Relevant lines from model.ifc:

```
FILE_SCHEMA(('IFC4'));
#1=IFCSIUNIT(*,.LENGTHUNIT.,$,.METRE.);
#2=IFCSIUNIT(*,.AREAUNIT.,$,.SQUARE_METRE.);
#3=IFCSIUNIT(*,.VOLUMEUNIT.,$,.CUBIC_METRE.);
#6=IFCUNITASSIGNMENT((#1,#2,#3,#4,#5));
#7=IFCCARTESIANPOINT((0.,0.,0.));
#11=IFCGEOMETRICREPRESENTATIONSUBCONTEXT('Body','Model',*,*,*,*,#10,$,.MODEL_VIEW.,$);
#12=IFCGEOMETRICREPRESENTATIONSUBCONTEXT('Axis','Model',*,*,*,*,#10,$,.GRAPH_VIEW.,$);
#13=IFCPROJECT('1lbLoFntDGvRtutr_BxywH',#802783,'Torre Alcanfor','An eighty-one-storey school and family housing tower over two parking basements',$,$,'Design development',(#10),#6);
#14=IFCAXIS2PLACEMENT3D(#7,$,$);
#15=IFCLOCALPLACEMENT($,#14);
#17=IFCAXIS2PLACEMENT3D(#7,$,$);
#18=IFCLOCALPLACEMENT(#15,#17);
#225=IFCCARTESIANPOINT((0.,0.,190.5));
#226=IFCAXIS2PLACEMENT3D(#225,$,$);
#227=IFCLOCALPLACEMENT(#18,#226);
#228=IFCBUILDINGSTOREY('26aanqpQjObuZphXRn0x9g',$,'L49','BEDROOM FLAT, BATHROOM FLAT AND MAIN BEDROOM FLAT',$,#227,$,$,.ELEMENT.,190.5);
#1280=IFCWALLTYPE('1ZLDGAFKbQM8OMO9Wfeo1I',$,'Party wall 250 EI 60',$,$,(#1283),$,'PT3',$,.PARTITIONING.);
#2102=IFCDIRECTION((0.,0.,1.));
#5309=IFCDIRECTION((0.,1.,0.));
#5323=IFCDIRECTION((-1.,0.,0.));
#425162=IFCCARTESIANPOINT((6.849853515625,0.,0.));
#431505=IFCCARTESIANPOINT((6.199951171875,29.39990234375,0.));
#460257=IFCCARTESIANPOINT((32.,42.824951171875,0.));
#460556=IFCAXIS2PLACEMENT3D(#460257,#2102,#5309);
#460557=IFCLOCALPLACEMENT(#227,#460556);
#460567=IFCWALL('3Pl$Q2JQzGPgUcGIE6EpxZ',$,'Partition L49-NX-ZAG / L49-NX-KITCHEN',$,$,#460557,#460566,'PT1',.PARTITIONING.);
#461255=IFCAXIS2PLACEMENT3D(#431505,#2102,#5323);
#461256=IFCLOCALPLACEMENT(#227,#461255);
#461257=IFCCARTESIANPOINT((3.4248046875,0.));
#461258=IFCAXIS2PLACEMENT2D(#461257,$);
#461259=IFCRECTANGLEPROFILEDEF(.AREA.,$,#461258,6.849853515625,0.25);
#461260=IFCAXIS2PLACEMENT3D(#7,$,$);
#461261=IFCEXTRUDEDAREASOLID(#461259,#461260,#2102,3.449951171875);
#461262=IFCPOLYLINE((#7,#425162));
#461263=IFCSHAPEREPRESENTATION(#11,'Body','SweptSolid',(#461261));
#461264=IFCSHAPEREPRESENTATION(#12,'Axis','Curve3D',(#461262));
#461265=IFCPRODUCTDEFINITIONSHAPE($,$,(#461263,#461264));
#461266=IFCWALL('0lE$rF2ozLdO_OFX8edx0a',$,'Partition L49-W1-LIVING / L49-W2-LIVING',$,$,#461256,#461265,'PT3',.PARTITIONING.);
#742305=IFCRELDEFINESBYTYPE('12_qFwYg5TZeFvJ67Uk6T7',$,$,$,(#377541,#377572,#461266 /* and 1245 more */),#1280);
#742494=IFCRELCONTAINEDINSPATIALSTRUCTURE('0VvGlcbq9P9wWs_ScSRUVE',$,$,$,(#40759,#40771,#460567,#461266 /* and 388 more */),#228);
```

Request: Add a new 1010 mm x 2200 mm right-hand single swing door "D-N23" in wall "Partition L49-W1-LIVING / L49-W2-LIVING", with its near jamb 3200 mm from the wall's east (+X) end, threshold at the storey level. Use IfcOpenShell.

```python
import numpy as np
import ifcopenshell
import ifcopenshell.api.feature
import ifcopenshell.api.geometry
import ifcopenshell.api.root
import ifcopenshell.api.spatial
import ifcopenshell.geom
import ifcopenshell.util.element
import ifcopenshell.util.placement
import ifcopenshell.util.representation
import ifcopenshell.util.shape
import ifcopenshell.util.unit

model = ifcopenshell.open("model.ifc")
unit_scale = ifcopenshell.util.unit.calculate_unit_scale(model)
settings = ifcopenshell.geom.settings()


def volume(element):
    """Net volume in cubic metres, openings subtracted."""
    shape = ifcopenshell.geom.create_shape(settings, element)
    return ifcopenshell.util.shape.get_volume(shape.geometry)


wall = model.by_guid("0lE$rF2ozLdO_OFX8edx0a")
storey = ifcopenshell.util.element.get_container(wall, ifc_class="IfcBuildingStorey")
context = ifcopenshell.util.representation.get_context(model, "Model", "Body", "MODEL_VIEW")
before = volume(wall)

width, height, from_end, sill = 1.01, 2.2, 3.2, 0.0  # metres

# The wall runs along its own X axis, and the end named is its -X end.
wall_shape = ifcopenshell.geom.create_shape(settings, wall)
x, y, z = ifcopenshell.util.shape.get_vertices(wall_shape.geometry).T
start = x.min() + from_end
face, thickness = float(y.min()), float(y.max() - y.min())
wall_matrix = ifcopenshell.util.placement.get_local_placement(wall.ObjectPlacement)
level = ifcopenshell.util.placement.get_local_placement(storey.ObjectPlacement)[2, 3]


def in_wall(x, y):
    """Placement at x, y metres in the wall's axes, at sill height."""
    matrix = wall_matrix.copy()
    matrix[:, 3] = wall_matrix @ np.array([x / unit_scale, y / unit_scale, 0.0, 1.0])
    matrix[2, 3] = level + sill / unit_scale
    return matrix


# Opening: a box that overshoots both wall faces by 50 mm.
opening = ifcopenshell.api.root.create_entity(model, ifc_class="IfcOpeningElement", predefined_type="OPENING")
box = ifcopenshell.api.geometry.add_wall_representation(
    model, context=context, length=width, height=height, thickness=thickness + 0.1
)
ifcopenshell.api.geometry.assign_representation(model, product=opening, representation=box)
ifcopenshell.api.geometry.edit_object_placement(model, product=opening, matrix=in_wall(start, face - 0.05), is_si=False)
ifcopenshell.api.feature.add_feature(model, feature=opening, element=wall)

door = ifcopenshell.api.root.create_entity(model, ifc_class="IfcDoor", name="D-N23", predefined_type="DOOR")
door.OverallWidth, door.OverallHeight = width / unit_scale, height / unit_scale
door.OperationType = "SINGLE_SWING_RIGHT"
body = ifcopenshell.api.geometry.add_door_representation(
    model,
    context=context,
    overall_width=door.OverallWidth,
    overall_height=door.OverallHeight,
    operation_type="SINGLE_SWING_RIGHT",
    lining_properties={"LiningDepth": thickness / unit_scale, "ThresholdDepth": thickness / unit_scale},
)
ifcopenshell.api.geometry.assign_representation(model, product=door, representation=body)
ifcopenshell.api.spatial.assign_container(model, products=[door], relating_structure=storey)
ifcopenshell.api.feature.add_filling(model, opening=opening, element=door)

# The lining spans the wall, so the door starts at the wall face.
ifcopenshell.api.geometry.edit_object_placement(model, product=door, matrix=in_wall(start, face), is_si=False)

after = volume(wall)

print(f"wall volume {before:.3f} -> {after:.3f} m3")

model.write("model_rev.ifc")
```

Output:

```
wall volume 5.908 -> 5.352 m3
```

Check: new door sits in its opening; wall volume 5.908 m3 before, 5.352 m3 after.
